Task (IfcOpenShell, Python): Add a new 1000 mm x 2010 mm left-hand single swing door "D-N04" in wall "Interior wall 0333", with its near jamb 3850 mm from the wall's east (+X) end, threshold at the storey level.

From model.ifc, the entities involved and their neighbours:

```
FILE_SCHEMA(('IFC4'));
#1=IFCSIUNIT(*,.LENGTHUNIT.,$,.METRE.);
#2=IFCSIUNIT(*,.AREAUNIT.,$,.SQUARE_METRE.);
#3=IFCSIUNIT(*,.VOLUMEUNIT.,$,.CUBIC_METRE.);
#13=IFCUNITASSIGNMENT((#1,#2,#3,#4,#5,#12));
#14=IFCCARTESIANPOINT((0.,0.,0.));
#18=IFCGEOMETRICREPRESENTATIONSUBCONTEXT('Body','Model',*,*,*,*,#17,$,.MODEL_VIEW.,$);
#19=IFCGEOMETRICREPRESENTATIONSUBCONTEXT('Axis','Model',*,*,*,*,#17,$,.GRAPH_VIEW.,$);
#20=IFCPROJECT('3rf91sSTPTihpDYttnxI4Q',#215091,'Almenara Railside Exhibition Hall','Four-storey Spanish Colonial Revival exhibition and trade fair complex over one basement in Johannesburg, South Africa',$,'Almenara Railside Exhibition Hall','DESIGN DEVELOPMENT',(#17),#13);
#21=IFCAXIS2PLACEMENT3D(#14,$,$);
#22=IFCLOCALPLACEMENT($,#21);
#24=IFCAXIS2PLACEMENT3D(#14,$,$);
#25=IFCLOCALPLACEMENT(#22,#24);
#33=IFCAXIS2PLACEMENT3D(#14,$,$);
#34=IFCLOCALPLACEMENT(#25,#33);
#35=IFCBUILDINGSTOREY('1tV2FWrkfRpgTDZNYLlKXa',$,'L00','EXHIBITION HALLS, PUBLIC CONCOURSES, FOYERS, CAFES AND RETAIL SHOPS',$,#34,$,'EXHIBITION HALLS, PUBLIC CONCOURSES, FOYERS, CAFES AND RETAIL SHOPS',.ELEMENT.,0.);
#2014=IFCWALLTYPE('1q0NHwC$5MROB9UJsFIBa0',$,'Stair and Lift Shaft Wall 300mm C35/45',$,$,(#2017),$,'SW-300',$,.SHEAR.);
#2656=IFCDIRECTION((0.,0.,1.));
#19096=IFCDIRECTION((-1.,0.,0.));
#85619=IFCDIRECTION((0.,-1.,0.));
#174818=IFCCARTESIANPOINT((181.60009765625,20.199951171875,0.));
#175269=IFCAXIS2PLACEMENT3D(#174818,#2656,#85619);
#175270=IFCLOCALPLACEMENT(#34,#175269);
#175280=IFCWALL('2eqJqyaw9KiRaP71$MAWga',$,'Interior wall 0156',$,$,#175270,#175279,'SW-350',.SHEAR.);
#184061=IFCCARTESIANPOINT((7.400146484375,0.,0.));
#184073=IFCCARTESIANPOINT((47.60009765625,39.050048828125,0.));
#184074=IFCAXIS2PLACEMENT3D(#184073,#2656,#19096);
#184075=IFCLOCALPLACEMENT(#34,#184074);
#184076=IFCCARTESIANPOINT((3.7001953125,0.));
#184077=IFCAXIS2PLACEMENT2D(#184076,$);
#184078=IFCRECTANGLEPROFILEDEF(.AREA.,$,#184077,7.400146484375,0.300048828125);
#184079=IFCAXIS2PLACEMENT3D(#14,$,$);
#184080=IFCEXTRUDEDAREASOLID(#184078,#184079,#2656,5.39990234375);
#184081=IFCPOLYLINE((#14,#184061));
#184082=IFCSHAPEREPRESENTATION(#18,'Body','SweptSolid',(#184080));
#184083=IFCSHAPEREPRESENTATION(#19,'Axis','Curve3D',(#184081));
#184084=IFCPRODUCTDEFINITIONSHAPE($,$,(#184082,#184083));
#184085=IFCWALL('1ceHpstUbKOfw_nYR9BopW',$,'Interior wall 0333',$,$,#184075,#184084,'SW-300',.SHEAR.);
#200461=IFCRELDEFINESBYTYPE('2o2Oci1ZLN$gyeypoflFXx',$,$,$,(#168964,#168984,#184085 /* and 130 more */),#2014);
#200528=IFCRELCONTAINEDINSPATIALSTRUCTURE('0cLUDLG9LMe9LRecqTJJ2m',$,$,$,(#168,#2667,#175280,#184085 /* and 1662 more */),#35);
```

```python
import numpy as np
import ifcopenshell
import ifcopenshell.api.feature
import ifcopenshell.api.geometry
import ifcopenshell.api.root
import ifcopenshell.api.spatial
import ifcopenshell.geom
import ifcopenshell.util.element
import ifcopenshell.util.placement
import ifcopenshell.util.representation
import ifcopenshell.util.shape
import ifcopenshell.util.unit

model = ifcopenshell.open("model.ifc")
unit_scale = ifcopenshell.util.unit.calculate_unit_scale(model)
settings = ifcopenshell.geom.settings()


def volume(element):
    """Net volume in cubic metres, openings subtracted."""
    shape = ifcopenshell.geom.create_shape(settings, element)
    return ifcopenshell.util.shape.get_volume(shape.geometry)


wall = model.by_guid("1ceHpstUbKOfw_nYR9BopW")
storey = ifcopenshell.util.element.get_container(wall, ifc_class="IfcBuildingStorey")
context = ifcopenshell.util.representation.get_context(model, "Model", "Body", "MODEL_VIEW")
before = volume(wall)

width, height, from_end, sill = 1, 2.01, 3.85, 0.0  # metres

# The wall runs along its own X axis, and the end named is its -X end.
wall_shape = ifcopenshell.geom.create_shape(settings, wall)
x, y, z = ifcopenshell.util.shape.get_vertices(wall_shape.geometry).T
start = x.min() + from_end
face, thickness = float(y.min()), float(y.max() - y.min())
wall_matrix = ifcopenshell.util.placement.get_local_placement(wall.ObjectPlacement)
level = ifcopenshell.util.placement.get_local_placement(storey.ObjectPlacement)[2, 3]


def in_wall(x, y):
    """Placement at x, y metres in the wall's axes, at sill height."""
    matrix = wall_matrix.copy()
    matrix[:, 3] = wall_matrix @ np.array([x / unit_scale, y / unit_scale, 0.0, 1.0])
    matrix[2, 3] = level + sill / unit_scale
    return matrix


# Opening: a box that overshoots both wall faces by 50 mm.
opening = ifcopenshell.api.root.create_entity(model, ifc_class="IfcOpeningElement", predefined_type="OPENING")
box = ifcopenshell.api.geometry.add_wall_representation(
    model, context=context, length=width, height=height, thickness=thickness + 0.1
)
ifcopenshell.api.geometry.assign_representation(model, product=opening, representation=box)
ifcopenshell.api.geometry.edit_object_placement(model, product=opening, matrix=in_wall(start, face - 0.05), is_si=False)
ifcopenshell.api.feature.add_feature(model, feature=opening, element=wall)

door = ifcopenshell.api.root.create_entity(model, ifc_class="IfcDoor", name="D-N04", predefined_type="DOOR")
door.OverallWidth, door.OverallHeight = width / unit_scale, height / unit_scale
door.OperationType = "SINGLE_SWING_LEFT"
body = ifcopenshell.api.geometry.add_door_representation(
    model,
    context=context,
    overall_width=door.OverallWidth,
    overall_height=door.OverallHeight,
    operation_type="SINGLE_SWING_LEFT",
    lining_properties={"LiningDepth": thickness / unit_scale, "ThresholdDepth": thickness / unit_scale},
)
ifcopenshell.api.geometry.assign_representation(model, product=door, representation=body)
ifcopenshell.api.spatial.assign_container(model, products=[door], relating_structure=storey)
ifcopenshell.api.feature.add_filling(model, opening=opening, element=door)

# The lining spans the wall, so the door starts at the wall face.
ifcopenshell.api.geometry.edit_object_placement(model, product=door, matrix=in_wall(start, face), is_si=False)

after = volume(wall)

print(f"wall volume {before:.3f} -> {after:.3f} m3")

model.write("model_edited.ifc")
```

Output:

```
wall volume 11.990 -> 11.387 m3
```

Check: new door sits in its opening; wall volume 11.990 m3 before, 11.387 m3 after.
